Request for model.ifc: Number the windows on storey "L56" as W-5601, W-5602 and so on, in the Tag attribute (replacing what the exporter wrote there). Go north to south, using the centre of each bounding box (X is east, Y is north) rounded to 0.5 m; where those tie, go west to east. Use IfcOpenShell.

First a look at what the model holds.

```python
import ifcopenshell
import ifcopenshell.util.element
import ifcopenshell.util.placement

model = ifcopenshell.open("model.ifc")
print(model.schema)
storey = next(s for s in model.by_type("IfcBuildingStorey") if s.Name == "L56")
windows = [e for e in ifcopenshell.util.element.get_decomposition(storey) if e.is_a("IfcWindow")]
for e in sorted(windows, key=lambda e: e.id()):
    origin = ifcopenshell.util.placement.get_local_placement(e.ObjectPlacement)[:3, 3]
    print(e.id(), e.Tag, e.Name, origin.round(2) + 0.0, sep=" | ")
```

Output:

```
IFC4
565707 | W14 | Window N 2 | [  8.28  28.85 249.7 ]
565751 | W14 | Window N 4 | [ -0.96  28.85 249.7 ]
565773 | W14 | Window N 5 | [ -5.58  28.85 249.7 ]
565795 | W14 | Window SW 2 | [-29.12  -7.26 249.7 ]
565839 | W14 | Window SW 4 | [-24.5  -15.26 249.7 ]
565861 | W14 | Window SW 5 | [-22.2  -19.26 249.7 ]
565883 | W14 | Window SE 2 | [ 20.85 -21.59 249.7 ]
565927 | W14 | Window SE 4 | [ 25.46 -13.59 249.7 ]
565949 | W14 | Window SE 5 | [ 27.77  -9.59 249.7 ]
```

```python
import ifcopenshell
import ifcopenshell.geom
import ifcopenshell.util.element
import ifcopenshell.util.shape

model = ifcopenshell.open("model.ifc")
settings = ifcopenshell.geom.settings()
settings.set("use-world-coords", True)


def centre(element):
    shape = ifcopenshell.geom.create_shape(settings, element)
    return ifcopenshell.util.shape.get_bbox_centroid(shape.geometry)


storey = next(s for s in model.by_type("IfcBuildingStorey") if s.Name == "L56")
windows = [e for e in ifcopenshell.util.element.get_decomposition(storey) if e.is_a("IfcWindow")]

# Insertion points can sit at a corner or the storey origin, so sort by the geometry (in metres).
centres = {e: centre(e) for e in windows}
windows.sort(key=lambda e: (-round(centres[e][1] / 0.5), centres[e][0]))

for i, e in enumerate(windows, start=1):
    number = f"W-56{i:02d}"
    e.Tag = number
    print(e.id(), number)

model.write("model_edited.ifc")
```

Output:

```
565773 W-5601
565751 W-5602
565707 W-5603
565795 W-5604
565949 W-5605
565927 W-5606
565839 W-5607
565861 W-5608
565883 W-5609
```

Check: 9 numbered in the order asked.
